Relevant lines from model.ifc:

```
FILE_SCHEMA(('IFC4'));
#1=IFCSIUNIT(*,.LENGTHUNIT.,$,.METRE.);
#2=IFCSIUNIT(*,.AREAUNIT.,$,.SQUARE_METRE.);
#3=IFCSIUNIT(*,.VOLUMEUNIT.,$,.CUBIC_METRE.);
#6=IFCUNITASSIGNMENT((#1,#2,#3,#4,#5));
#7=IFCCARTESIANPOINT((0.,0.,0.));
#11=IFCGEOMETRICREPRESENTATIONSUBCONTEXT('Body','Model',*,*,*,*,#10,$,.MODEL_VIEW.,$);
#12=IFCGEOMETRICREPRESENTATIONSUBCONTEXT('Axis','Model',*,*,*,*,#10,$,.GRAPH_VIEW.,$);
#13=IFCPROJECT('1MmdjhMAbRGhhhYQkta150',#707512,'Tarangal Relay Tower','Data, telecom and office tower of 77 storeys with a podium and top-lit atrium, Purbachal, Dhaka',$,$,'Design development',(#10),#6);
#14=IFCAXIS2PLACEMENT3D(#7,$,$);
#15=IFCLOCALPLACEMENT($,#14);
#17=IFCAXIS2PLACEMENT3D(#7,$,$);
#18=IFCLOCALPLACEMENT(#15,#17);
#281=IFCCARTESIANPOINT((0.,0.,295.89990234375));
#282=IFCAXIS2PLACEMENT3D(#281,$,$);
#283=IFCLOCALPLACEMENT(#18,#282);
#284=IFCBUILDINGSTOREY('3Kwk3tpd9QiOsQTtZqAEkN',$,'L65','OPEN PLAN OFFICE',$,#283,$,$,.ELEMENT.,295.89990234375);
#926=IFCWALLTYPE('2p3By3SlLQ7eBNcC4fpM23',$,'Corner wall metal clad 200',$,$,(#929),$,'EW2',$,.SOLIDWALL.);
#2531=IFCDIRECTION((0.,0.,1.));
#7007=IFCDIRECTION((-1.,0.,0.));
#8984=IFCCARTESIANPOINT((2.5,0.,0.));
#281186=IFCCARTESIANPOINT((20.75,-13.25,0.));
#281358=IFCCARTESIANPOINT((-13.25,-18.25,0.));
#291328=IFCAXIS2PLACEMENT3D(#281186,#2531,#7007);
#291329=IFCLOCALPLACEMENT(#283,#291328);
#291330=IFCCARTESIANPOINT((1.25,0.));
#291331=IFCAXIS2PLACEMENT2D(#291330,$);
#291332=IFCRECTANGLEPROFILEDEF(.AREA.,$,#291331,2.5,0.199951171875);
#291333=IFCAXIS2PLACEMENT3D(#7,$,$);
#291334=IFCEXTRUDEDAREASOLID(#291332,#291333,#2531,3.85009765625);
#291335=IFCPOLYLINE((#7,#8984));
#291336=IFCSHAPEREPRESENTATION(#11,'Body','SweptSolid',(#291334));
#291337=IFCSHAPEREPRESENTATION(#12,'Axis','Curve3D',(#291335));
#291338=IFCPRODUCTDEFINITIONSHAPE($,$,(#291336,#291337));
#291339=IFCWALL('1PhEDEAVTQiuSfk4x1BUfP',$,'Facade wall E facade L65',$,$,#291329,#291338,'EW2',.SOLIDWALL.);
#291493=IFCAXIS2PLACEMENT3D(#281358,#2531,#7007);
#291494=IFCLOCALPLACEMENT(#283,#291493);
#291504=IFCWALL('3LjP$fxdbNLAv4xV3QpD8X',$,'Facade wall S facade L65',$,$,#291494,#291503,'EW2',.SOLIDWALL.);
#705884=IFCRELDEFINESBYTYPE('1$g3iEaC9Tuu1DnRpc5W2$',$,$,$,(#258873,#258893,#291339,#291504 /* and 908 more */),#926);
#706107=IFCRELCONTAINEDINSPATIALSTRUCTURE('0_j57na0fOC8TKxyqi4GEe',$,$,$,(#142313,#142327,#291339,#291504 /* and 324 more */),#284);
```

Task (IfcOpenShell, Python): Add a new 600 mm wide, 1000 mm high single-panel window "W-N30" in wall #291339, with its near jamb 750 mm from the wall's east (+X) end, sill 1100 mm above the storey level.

```python
import numpy as np
import ifcopenshell
import ifcopenshell.api.feature
import ifcopenshell.api.geometry
import ifcopenshell.api.root
import ifcopenshell.api.spatial
import ifcopenshell.geom
import ifcopenshell.util.element
import ifcopenshell.util.placement
import ifcopenshell.util.representation
import ifcopenshell.util.shape
import ifcopenshell.util.unit

model = ifcopenshell.open("model.ifc")
unit_scale = ifcopenshell.util.unit.calculate_unit_scale(model)
settings = ifcopenshell.geom.settings()


def volume(element):
    """Net volume in cubic metres, openings subtracted."""
    shape = ifcopenshell.geom.create_shape(settings, element)
    return ifcopenshell.util.shape.get_volume(shape.geometry)


wall = model.by_guid("1PhEDEAVTQiuSfk4x1BUfP")
storey = ifcopenshell.util.element.get_container(wall, ifc_class="IfcBuildingStorey")
context = ifcopenshell.util.representation.get_context(model, "Model", "Body", "MODEL_VIEW")
before = volume(wall)

width, height, from_end, sill = 0.6, 1, 0.75, 1.1  # metres

# The wall runs along its own X axis, and the end named is its -X end.
wall_shape = ifcopenshell.geom.create_shape(settings, wall)
x, y, z = ifcopenshell.util.shape.get_vertices(wall_shape.geometry).T
start = x.min() + from_end
face, thickness = float(y.min()), float(y.max() - y.min())
wall_matrix = ifcopenshell.util.placement.get_local_placement(wall.ObjectPlacement)
level = ifcopenshell.util.placement.get_local_placement(storey.ObjectPlacement)[2, 3]


def in_wall(x, y):
    """Placement at x, y metres in the wall's axes, at sill height."""
    matrix = wall_matrix.copy()
    matrix[:, 3] = wall_matrix @ np.array([x / unit_scale, y / unit_scale, 0.0, 1.0])
    matrix[2, 3] = level + sill / unit_scale
    return matrix


# Opening: a box that overshoots both wall faces by 50 mm.
opening = ifcopenshell.api.root.create_entity(model, ifc_class="IfcOpeningElement", predefined_type="OPENING")
box = ifcopenshell.api.geometry.add_wall_representation(
    model, context=context, length=width, height=height, thickness=thickness + 0.1
)
ifcopenshell.api.geometry.assign_representation(model, product=opening, representation=box)
ifcopenshell.api.geometry.edit_object_placement(model, product=opening, matrix=in_wall(start, face - 0.05), is_si=False)
ifcopenshell.api.feature.add_feature(model, feature=opening, element=wall)

window = ifcopenshell.api.root.create_entity(model, ifc_class="IfcWindow", name="W-N30", predefined_type="WINDOW")
window.OverallWidth, window.OverallHeight = width / unit_scale, height / unit_scale
window.PartitioningType = "SINGLE_PANEL"
body = ifcopenshell.api.geometry.add_window_representation(
    model,
    context=context,
    overall_width=window.OverallWidth,
    overall_height=window.OverallHeight,
    partition_type="SINGLE_PANEL",
)
ifcopenshell.api.geometry.assign_representation(model, product=window, representation=body)
ifcopenshell.api.spatial.assign_container(model, products=[window], relating_structure=storey)
ifcopenshell.api.feature.add_filling(model, opening=opening, element=window)

# Centre the window in the wall's thickness.
ifcopenshell.api.geometry.edit_object_placement(model, product=window, matrix=in_wall(start, face), is_si=False)
window_shape = ifcopenshell.geom.create_shape(settings, window)
depth = ifcopenshell.util.shape.get_vertices(window_shape.geometry)[:, 1]
offset = face + thickness / 2 - (depth.min() + depth.max()) / 2
ifcopenshell.api.geometry.edit_object_placement(model, product=window, matrix=in_wall(start, offset), is_si=False)

after = volume(wall)

print(f"wall volume {before:.3f} -> {after:.3f} m3")

model.write("model-out.ifc")
```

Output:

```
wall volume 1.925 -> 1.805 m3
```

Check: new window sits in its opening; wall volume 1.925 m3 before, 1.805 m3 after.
